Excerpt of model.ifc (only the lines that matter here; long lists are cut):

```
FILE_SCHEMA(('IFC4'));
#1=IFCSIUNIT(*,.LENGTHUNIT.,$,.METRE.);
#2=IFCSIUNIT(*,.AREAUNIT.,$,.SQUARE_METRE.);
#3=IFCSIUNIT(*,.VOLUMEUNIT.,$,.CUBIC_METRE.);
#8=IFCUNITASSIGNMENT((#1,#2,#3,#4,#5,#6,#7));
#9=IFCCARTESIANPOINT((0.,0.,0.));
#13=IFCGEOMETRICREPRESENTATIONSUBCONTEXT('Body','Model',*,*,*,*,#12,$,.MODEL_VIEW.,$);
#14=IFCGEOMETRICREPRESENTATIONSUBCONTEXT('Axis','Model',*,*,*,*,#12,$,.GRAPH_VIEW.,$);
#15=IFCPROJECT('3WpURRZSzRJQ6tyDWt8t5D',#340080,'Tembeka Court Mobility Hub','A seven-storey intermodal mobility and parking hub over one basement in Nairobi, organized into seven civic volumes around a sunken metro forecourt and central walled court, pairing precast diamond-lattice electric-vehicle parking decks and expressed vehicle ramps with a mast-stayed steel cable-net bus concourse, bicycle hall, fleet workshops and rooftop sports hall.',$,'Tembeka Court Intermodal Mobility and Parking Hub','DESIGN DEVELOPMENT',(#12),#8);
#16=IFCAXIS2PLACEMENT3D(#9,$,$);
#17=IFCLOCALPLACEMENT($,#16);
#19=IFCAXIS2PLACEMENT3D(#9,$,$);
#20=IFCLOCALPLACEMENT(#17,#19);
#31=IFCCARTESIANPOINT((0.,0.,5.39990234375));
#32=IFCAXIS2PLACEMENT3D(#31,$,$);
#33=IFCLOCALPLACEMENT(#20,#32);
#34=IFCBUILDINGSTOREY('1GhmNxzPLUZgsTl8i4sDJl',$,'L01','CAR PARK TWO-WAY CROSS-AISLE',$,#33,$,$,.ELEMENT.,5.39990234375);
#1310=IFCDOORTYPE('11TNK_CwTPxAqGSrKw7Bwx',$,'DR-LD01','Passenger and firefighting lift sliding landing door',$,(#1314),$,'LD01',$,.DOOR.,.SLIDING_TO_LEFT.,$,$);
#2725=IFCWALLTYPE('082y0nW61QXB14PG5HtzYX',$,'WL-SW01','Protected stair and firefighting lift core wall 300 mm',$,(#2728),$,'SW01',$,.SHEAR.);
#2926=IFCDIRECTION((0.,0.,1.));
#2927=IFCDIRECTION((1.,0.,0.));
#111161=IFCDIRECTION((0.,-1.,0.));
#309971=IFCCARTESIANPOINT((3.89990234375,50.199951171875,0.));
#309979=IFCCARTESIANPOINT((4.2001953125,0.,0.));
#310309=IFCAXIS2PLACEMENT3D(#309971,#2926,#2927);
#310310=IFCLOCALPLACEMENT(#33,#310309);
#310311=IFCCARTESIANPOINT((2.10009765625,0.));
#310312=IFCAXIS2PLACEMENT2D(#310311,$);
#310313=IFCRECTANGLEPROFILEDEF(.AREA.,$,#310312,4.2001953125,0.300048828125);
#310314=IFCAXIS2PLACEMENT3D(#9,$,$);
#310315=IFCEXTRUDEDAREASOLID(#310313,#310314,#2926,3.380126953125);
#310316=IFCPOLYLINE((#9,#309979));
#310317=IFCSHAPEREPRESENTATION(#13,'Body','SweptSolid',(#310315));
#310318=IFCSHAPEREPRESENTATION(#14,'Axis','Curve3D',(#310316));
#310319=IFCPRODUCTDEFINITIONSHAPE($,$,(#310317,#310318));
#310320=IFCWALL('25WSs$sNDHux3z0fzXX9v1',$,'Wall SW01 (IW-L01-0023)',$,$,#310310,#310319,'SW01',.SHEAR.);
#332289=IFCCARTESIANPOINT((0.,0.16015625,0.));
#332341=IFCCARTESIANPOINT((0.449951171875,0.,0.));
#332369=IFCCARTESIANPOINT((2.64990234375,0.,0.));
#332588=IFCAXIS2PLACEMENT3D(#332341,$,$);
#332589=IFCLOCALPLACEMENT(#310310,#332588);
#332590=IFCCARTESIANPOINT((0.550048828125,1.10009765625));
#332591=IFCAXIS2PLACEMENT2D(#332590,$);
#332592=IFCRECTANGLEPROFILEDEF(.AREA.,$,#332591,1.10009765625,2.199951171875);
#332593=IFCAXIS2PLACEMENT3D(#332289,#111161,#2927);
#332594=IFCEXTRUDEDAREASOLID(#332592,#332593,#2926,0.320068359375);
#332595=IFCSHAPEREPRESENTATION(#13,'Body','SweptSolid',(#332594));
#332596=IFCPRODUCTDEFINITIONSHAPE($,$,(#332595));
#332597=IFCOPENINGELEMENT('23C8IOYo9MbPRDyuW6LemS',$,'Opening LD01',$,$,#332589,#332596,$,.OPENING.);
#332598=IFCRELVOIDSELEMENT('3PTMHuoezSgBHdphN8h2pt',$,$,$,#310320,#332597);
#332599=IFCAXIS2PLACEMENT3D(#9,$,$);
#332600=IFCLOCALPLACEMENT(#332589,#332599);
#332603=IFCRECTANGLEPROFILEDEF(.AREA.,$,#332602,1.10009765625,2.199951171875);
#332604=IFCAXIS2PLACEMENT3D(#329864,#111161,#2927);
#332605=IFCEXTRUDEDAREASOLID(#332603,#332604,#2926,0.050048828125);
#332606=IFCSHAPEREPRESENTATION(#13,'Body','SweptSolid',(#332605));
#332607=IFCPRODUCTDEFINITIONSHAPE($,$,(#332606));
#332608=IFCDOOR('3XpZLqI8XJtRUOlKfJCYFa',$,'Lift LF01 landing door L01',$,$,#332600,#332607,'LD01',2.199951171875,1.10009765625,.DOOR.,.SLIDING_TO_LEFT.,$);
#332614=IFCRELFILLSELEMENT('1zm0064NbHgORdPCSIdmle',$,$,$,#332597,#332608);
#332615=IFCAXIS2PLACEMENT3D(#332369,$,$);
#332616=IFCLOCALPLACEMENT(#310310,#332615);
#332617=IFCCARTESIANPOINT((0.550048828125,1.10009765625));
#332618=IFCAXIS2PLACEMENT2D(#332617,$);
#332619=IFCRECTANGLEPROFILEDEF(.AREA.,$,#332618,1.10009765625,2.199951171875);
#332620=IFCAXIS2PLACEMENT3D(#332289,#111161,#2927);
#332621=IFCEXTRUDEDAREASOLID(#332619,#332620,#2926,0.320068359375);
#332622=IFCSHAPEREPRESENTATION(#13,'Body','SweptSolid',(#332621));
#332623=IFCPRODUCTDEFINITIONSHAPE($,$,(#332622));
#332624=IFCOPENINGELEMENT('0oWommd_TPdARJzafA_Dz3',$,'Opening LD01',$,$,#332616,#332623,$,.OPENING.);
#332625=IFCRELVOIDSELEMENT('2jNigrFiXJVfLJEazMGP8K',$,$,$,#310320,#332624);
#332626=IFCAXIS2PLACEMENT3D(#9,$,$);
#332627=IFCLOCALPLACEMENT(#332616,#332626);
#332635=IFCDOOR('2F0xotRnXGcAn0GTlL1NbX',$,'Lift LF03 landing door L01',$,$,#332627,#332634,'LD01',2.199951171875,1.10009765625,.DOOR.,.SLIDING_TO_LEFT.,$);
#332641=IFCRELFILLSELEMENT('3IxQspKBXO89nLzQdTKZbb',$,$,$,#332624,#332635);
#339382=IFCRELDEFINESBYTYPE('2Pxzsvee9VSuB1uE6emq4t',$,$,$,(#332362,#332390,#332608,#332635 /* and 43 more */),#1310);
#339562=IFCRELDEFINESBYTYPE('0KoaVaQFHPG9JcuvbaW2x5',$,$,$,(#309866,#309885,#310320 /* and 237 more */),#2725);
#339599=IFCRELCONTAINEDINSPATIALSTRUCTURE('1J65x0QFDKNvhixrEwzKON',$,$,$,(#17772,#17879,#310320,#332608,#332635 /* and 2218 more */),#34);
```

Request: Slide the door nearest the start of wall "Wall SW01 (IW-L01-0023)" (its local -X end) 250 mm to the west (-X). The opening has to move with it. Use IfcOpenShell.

```python
import ifcopenshell
import ifcopenshell.api.geometry
import ifcopenshell.util.placement

model = ifcopenshell.open("model.ifc")

door = model.by_guid("3XpZLqI8XJtRUOlKfJCYFa")
opening = door.FillsVoids[0].RelatingOpeningElement
wall = opening.VoidsElements[0].RelatingBuildingElement

wall_matrix = ifcopenshell.util.placement.get_local_placement(wall.ObjectPlacement)
shift = wall_matrix[:3, 0] * -0.25
before = ifcopenshell.util.placement.get_local_placement(door.ObjectPlacement)[:3, 3].copy()

# The door is placed relative to its opening, so it follows when the opening moves.
matrix = ifcopenshell.util.placement.get_local_placement(opening.ObjectPlacement)
matrix[:3, 3] += shift
ifcopenshell.api.geometry.edit_object_placement(
    model, product=opening, matrix=matrix, is_si=False, should_transform_children=True
)

after = ifcopenshell.util.placement.get_local_placement(door.ObjectPlacement)[:3, 3]
print("door moved by", (after - before).round(3) + 0.0)

model.write("model_updated.ifc")
```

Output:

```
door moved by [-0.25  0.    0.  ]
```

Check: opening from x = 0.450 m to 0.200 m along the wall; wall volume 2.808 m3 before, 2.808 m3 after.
